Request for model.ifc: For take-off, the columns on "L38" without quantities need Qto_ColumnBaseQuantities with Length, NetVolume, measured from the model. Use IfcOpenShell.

First a look at what the model holds.

```python
import ifcopenshell
import ifcopenshell.util.element
import ifcopenshell.util.unit

model = ifcopenshell.open("model.ifc")
print(model.schema)
for unit_type in ("LENGTHUNIT", "AREAUNIT", "VOLUMEUNIT"):
    print(unit_type, ifcopenshell.util.unit.calculate_unit_scale(model, unit_type))
storey = next(s for s in model.by_type("IfcBuildingStorey") if s.Name == "L38")
columns = [e for e in ifcopenshell.util.element.get_decomposition(storey) if e.is_a("IfcColumn")]
for e in sorted(columns, key=lambda e: e.id()):
    print(e.id(), e.is_a(), e.Name, list(ifcopenshell.util.element.get_psets(e, qtos_only=True)), sep=" | ")
```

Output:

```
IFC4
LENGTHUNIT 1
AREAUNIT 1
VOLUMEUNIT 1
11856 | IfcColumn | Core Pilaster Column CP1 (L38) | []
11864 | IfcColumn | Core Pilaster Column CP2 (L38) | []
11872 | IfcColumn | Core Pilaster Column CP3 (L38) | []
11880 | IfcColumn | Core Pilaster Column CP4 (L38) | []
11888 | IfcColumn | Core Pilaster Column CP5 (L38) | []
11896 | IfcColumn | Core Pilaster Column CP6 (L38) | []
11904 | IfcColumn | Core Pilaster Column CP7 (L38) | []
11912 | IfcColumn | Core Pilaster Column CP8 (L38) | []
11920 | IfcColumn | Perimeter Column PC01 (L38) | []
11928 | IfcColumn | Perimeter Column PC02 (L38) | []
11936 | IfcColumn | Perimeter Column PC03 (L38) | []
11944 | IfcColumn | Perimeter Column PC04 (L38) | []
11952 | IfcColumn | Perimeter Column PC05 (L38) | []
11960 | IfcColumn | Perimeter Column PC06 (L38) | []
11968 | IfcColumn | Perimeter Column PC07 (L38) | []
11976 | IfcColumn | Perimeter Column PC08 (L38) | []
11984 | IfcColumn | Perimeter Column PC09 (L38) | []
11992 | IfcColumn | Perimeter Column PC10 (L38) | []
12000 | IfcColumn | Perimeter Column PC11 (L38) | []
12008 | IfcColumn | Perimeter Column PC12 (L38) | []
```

```python
import ifcopenshell
import ifcopenshell.api.pset
import ifcopenshell.geom
import ifcopenshell.util.element
import ifcopenshell.util.shape
import ifcopenshell.util.unit

model = ifcopenshell.open("model.ifc")
unit_scale = ifcopenshell.util.unit.calculate_unit_scale(model)
volume_scale = ifcopenshell.util.unit.calculate_unit_scale(model, "VOLUMEUNIT")
settings = ifcopenshell.geom.settings()

storey = next(s for s in model.by_type("IfcBuildingStorey") if s.Name == "L38")
columns = [e for e in ifcopenshell.util.element.get_decomposition(storey) if e.is_a("IfcColumn")]

for e in sorted(columns, key=lambda e: e.id()):
    if ifcopenshell.util.element.get_psets(e, qtos_only=True, should_inherit=False):
        continue
    # Geometry comes back in metres, in the element's own axes.
    shape = ifcopenshell.geom.create_shape(settings, e)
    values = {
        "Length": ifcopenshell.util.shape.get_z(shape.geometry) / unit_scale,
        "NetVolume": ifcopenshell.util.shape.get_volume(shape.geometry) / volume_scale,
    }
    qto = ifcopenshell.api.pset.add_qto(model, product=e, name="Qto_ColumnBaseQuantities")
    ifcopenshell.api.pset.edit_qto(model, qto=qto, properties=values)
    print(e.id(), {k: round(v, 3) for k, v in values.items()})

model.write("model_v2.ifc")
```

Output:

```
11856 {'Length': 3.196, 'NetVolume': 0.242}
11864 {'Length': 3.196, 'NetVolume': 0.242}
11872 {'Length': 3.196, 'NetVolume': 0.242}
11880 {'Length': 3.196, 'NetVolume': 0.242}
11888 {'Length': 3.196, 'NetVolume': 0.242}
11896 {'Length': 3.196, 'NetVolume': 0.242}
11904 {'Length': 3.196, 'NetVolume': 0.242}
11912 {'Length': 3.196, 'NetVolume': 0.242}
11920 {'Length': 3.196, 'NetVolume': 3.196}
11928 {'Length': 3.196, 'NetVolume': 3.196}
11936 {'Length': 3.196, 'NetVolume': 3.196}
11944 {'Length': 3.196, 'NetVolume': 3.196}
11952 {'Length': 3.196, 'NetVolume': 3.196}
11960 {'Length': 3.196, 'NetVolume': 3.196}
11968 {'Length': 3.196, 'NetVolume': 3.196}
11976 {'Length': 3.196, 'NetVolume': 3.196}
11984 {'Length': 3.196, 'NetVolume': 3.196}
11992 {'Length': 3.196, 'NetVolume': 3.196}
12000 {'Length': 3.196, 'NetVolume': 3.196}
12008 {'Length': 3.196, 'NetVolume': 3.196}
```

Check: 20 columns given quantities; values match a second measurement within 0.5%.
